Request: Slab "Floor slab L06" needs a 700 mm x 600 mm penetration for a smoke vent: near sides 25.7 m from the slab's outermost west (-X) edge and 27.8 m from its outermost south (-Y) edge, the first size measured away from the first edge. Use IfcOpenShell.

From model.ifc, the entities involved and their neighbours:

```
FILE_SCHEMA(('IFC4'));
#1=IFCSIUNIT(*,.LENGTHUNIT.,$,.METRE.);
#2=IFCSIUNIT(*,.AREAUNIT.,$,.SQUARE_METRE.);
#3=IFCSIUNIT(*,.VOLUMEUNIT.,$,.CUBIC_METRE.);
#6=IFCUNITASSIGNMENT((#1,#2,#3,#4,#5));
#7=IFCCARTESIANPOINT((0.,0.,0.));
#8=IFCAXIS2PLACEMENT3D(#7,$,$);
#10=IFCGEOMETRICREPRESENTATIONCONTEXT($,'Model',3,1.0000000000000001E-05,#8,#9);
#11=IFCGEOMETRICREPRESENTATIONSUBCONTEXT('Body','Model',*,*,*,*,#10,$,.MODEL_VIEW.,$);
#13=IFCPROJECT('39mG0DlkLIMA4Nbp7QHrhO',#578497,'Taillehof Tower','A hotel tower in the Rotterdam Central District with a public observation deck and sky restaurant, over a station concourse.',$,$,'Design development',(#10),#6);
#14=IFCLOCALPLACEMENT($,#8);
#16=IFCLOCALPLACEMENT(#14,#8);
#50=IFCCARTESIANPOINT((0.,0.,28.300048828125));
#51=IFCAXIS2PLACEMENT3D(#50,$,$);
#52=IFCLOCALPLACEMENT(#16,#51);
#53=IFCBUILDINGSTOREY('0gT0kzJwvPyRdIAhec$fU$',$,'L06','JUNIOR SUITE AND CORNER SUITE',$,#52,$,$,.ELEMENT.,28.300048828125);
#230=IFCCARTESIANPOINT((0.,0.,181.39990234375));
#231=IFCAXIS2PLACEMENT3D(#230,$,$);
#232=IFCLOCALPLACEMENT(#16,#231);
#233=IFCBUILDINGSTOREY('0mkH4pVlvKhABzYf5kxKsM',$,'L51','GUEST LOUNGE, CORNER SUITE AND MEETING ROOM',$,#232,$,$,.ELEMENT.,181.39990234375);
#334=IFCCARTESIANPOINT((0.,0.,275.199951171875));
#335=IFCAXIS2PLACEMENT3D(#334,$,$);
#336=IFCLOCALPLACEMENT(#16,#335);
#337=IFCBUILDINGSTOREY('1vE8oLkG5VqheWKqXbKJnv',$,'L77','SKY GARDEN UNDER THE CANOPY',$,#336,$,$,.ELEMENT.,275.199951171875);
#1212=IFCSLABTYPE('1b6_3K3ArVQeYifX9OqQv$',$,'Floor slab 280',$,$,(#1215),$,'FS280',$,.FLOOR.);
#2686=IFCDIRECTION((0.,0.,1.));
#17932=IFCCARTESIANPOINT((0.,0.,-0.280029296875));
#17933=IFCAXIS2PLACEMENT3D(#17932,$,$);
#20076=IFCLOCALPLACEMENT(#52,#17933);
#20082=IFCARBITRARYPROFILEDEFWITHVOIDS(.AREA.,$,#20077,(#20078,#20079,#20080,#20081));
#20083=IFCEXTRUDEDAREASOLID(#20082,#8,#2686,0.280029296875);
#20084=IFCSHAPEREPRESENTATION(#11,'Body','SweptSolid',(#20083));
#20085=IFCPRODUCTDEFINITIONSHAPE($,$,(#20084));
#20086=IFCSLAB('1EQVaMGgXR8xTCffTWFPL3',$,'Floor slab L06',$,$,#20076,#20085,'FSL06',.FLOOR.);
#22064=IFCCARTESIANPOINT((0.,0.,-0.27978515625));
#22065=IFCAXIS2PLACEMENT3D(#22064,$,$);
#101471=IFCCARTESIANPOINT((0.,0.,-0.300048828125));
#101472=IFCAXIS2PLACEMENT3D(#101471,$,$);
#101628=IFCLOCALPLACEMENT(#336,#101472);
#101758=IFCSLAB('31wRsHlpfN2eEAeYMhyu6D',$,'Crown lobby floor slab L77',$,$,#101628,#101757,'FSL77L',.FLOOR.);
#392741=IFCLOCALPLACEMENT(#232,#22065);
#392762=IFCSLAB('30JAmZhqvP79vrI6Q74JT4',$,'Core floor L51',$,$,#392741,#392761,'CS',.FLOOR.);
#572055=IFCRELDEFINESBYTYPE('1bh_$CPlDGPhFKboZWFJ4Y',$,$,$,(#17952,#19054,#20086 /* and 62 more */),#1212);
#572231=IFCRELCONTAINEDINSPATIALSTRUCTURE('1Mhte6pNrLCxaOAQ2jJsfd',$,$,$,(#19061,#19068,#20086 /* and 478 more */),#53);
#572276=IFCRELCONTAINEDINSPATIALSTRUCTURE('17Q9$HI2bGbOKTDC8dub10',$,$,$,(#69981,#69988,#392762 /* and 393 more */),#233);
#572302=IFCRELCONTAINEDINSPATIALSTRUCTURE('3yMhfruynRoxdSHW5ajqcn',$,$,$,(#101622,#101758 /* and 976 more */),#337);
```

```python
import numpy as np
import ifcopenshell
import ifcopenshell.api.feature
import ifcopenshell.api.geometry
import ifcopenshell.api.root
import ifcopenshell.geom
import ifcopenshell.util.placement
import ifcopenshell.util.representation
import ifcopenshell.util.shape
import ifcopenshell.util.unit

model = ifcopenshell.open("model.ifc")
unit_scale = ifcopenshell.util.unit.calculate_unit_scale(model)
settings = ifcopenshell.geom.settings()


def volume(element):
    """Net volume in cubic metres, openings subtracted."""
    shape = ifcopenshell.geom.create_shape(settings, element)
    return ifcopenshell.util.shape.get_volume(shape.geometry)


slab = model.by_guid("1EQVaMGgXR8xTCffTWFPL3")
before = volume(slab)

# Extent in the slab's own axes, in metres. The edges named are its -X and -Y sides.
slab_shape = ifcopenshell.geom.create_shape(settings, slab)
vertices = ifcopenshell.util.shape.get_vertices(slab_shape.geometry)
x_min, y_min, bottom = vertices.min(axis=0)
top = vertices[:, 2].max()

opening = ifcopenshell.api.root.create_entity(model, ifc_class="IfcOpeningElement", name="Smoke vent opening", predefined_type="OPENING")
context = ifcopenshell.util.representation.get_context(model, "Model", "Body", "MODEL_VIEW")
width, depth = 0.7, 0.6
outline = [(0.0, 0.0), (width, 0.0), (width, depth), (0.0, depth), (0.0, 0.0)]
# Overshoot both faces by 50 mm so the cut is clean.
shape = ifcopenshell.api.geometry.add_slab_representation(
    model, context=context, depth=top - bottom + 0.1, polyline=outline
)
ifcopenshell.api.geometry.assign_representation(model, product=opening, representation=shape)

matrix = ifcopenshell.util.placement.get_local_placement(slab.ObjectPlacement)
matrix[:, 3] = matrix @ np.append(np.array([x_min + 25.7, y_min + 27.8, bottom - 0.05]) / unit_scale, 1.0)
ifcopenshell.api.geometry.edit_object_placement(model, product=opening, matrix=matrix, is_si=False)
ifcopenshell.api.feature.add_feature(model, feature=opening, element=slab)

after = volume(slab)

print(f"slab volume {before:.3f} -> {after:.3f} m3")

model.write("model_rev.ifc")
```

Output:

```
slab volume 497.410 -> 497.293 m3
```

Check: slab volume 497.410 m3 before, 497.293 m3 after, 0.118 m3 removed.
